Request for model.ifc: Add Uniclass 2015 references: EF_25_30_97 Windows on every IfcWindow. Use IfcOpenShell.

First a look at what the model holds.

```python
import ifcopenshell

model = ifcopenshell.open("model.ifc")
print(model.schema)
print("classifications:", [c.Name for c in model.by_type("IfcClassification")])
for ifc_class in ("IfcDoor", "IfcRoof", "IfcStair", "IfcWall", "IfcWindow"):
    print(ifc_class, len(model.by_type(ifc_class)))
```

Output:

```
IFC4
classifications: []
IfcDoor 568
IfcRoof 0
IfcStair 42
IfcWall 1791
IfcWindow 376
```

```python
import ifcopenshell
import ifcopenshell.api.classification

model = ifcopenshell.open("model.ifc")

system = ifcopenshell.api.classification.add_classification(model, classification="Uniclass 2015")

codes = {
    "IfcWindow": ("EF_25_30_97", "Windows"),
}
for ifc_class, (code, name) in codes.items():
    products = model.by_type(ifc_class)
    ifcopenshell.api.classification.add_reference(
        model, products=products, classification=system, identification=code, name=name
    )
    print(code, len(products))

model.write("model_rev.ifc")
```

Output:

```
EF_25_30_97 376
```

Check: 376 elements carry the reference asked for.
